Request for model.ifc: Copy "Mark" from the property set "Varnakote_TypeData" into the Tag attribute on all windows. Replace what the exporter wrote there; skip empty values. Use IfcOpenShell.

First a look at what the model holds.

```python
import ifcopenshell
import ifcopenshell.util.element

model = ifcopenshell.open("model.ifc")
print(model.schema)
windows = model.by_type("IfcWindow")
print(len(windows), "windows")
for e in windows[:8]:
    source = ifcopenshell.util.element.get_pset(e, "Varnakote_TypeData", "Mark")
    target = e.Tag
    print(e.id(), repr(source), repr(target), sep=" | ")
```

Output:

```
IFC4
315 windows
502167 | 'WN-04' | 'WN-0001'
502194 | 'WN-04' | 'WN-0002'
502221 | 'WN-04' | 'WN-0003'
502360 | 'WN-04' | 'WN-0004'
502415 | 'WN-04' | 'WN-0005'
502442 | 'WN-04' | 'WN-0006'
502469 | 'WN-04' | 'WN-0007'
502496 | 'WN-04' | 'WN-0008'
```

```python
import ifcopenshell
import ifcopenshell.util.element

model = ifcopenshell.open("model.ifc")

count = 0
for e in model.by_type("IfcWindow"):
    value = ifcopenshell.util.element.get_pset(e, "Varnakote_TypeData", "Mark")
    current = e.Tag
    if not value or not value.strip() or current == value:
        continue
    e.Tag = value
    count += 1

print(count, "windows updated")

model.write("model_rev.ifc")
```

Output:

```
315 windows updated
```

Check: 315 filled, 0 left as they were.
